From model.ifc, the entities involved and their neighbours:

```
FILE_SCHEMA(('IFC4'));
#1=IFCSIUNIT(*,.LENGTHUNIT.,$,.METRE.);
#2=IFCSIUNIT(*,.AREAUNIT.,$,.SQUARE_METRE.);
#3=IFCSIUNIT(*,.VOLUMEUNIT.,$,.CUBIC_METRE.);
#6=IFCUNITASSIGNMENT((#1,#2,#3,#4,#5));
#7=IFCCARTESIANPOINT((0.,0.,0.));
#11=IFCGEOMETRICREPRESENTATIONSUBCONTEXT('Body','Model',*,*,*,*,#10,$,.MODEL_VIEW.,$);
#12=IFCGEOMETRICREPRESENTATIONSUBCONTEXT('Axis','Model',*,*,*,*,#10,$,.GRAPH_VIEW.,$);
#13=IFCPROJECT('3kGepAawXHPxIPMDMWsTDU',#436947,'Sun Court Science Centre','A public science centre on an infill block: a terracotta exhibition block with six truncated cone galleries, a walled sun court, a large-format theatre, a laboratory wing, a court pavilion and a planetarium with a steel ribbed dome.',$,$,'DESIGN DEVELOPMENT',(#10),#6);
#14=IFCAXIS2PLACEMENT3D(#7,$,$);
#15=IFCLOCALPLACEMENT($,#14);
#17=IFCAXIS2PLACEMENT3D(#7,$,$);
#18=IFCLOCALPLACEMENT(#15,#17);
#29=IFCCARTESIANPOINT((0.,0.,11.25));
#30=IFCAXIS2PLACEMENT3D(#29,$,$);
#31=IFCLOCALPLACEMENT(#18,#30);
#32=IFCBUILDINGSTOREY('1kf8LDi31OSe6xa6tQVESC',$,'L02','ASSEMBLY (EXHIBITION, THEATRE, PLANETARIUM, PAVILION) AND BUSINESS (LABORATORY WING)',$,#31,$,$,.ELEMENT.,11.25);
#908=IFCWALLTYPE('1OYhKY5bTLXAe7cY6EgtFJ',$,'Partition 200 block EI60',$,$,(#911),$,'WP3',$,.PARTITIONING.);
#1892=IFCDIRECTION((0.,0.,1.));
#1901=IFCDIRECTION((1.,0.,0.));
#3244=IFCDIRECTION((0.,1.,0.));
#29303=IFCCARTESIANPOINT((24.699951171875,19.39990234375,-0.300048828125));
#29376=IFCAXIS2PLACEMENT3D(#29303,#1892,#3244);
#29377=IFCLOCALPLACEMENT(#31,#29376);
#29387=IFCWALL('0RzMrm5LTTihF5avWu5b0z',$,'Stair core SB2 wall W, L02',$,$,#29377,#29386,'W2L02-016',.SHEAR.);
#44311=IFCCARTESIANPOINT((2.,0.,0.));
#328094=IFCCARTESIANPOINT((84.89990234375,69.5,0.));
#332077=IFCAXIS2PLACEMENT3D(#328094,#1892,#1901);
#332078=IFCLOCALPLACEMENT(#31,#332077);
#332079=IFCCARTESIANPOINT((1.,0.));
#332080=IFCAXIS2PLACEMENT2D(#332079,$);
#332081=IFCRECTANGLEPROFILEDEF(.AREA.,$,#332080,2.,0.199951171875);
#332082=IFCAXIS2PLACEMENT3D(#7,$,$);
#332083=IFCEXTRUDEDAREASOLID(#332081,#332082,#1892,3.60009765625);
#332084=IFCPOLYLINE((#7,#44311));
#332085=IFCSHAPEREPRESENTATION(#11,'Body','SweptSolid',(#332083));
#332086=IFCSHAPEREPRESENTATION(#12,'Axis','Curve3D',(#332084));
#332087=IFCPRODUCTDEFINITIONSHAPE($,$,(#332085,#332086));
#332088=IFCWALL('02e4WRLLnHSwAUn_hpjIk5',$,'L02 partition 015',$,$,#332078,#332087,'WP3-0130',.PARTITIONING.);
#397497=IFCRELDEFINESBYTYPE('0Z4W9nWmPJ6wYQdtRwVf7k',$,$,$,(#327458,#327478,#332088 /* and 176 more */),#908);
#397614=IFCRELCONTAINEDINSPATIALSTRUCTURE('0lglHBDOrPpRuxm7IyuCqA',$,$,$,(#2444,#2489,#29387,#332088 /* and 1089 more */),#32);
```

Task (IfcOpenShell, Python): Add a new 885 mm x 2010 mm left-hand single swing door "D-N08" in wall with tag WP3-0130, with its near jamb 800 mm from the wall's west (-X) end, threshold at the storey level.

```python
import numpy as np
import ifcopenshell
import ifcopenshell.api.feature
import ifcopenshell.api.geometry
import ifcopenshell.api.root
import ifcopenshell.api.spatial
import ifcopenshell.geom
import ifcopenshell.util.element
import ifcopenshell.util.placement
import ifcopenshell.util.representation
import ifcopenshell.util.shape
import ifcopenshell.util.unit

model = ifcopenshell.open("model.ifc")
unit_scale = ifcopenshell.util.unit.calculate_unit_scale(model)
settings = ifcopenshell.geom.settings()


def volume(element):
    """Net volume in cubic metres, openings subtracted."""
    shape = ifcopenshell.geom.create_shape(settings, element)
    return ifcopenshell.util.shape.get_volume(shape.geometry)


wall = model.by_guid("02e4WRLLnHSwAUn_hpjIk5")
storey = ifcopenshell.util.element.get_container(wall, ifc_class="IfcBuildingStorey")
context = ifcopenshell.util.representation.get_context(model, "Model", "Body", "MODEL_VIEW")
before = volume(wall)

width, height, from_end, sill = 0.885, 2.01, 0.8, 0.0  # metres

# The wall runs along its own X axis, and the end named is its -X end.
wall_shape = ifcopenshell.geom.create_shape(settings, wall)
x, y, z = ifcopenshell.util.shape.get_vertices(wall_shape.geometry).T
start = x.min() + from_end
face, thickness = float(y.min()), float(y.max() - y.min())
wall_matrix = ifcopenshell.util.placement.get_local_placement(wall.ObjectPlacement)
level = ifcopenshell.util.placement.get_local_placement(storey.ObjectPlacement)[2, 3]


def in_wall(x, y):
    """Placement at x, y metres in the wall's axes, at sill height."""
    matrix = wall_matrix.copy()
    matrix[:, 3] = wall_matrix @ np.array([x / unit_scale, y / unit_scale, 0.0, 1.0])
    matrix[2, 3] = level + sill / unit_scale
    return matrix


# Opening: a box that overshoots both wall faces by 50 mm.
opening = ifcopenshell.api.root.create_entity(model, ifc_class="IfcOpeningElement", predefined_type="OPENING")
box = ifcopenshell.api.geometry.add_wall_representation(
    model, context=context, length=width, height=height, thickness=thickness + 0.1
)
ifcopenshell.api.geometry.assign_representation(model, product=opening, representation=box)
ifcopenshell.api.geometry.edit_object_placement(model, product=opening, matrix=in_wall(start, face - 0.05), is_si=False)
ifcopenshell.api.feature.add_feature(model, feature=opening, element=wall)

door = ifcopenshell.api.root.create_entity(model, ifc_class="IfcDoor", name="D-N08", predefined_type="DOOR")
door.OverallWidth, door.OverallHeight = width / unit_scale, height / unit_scale
door.OperationType = "SINGLE_SWING_LEFT"
body = ifcopenshell.api.geometry.add_door_representation(
    model,
    context=context,
    overall_width=door.OverallWidth,
    overall_height=door.OverallHeight,
    operation_type="SINGLE_SWING_LEFT",
    lining_properties={"LiningDepth": thickness / unit_scale, "ThresholdDepth": thickness / unit_scale},
)
ifcopenshell.api.geometry.assign_representation(model, product=door, representation=body)
ifcopenshell.api.spatial.assign_container(model, products=[door], relating_structure=storey)
ifcopenshell.api.feature.add_filling(model, opening=opening, element=door)

# The lining spans the wall, so the door starts at the wall face.
ifcopenshell.api.geometry.edit_object_placement(model, product=door, matrix=in_wall(start, face), is_si=False)

after = volume(wall)

print(f"wall volume {before:.3f} -> {after:.3f} m3")

model.write("model_updated.ifc")
```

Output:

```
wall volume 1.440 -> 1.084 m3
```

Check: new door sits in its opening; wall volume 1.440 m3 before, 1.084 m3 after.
